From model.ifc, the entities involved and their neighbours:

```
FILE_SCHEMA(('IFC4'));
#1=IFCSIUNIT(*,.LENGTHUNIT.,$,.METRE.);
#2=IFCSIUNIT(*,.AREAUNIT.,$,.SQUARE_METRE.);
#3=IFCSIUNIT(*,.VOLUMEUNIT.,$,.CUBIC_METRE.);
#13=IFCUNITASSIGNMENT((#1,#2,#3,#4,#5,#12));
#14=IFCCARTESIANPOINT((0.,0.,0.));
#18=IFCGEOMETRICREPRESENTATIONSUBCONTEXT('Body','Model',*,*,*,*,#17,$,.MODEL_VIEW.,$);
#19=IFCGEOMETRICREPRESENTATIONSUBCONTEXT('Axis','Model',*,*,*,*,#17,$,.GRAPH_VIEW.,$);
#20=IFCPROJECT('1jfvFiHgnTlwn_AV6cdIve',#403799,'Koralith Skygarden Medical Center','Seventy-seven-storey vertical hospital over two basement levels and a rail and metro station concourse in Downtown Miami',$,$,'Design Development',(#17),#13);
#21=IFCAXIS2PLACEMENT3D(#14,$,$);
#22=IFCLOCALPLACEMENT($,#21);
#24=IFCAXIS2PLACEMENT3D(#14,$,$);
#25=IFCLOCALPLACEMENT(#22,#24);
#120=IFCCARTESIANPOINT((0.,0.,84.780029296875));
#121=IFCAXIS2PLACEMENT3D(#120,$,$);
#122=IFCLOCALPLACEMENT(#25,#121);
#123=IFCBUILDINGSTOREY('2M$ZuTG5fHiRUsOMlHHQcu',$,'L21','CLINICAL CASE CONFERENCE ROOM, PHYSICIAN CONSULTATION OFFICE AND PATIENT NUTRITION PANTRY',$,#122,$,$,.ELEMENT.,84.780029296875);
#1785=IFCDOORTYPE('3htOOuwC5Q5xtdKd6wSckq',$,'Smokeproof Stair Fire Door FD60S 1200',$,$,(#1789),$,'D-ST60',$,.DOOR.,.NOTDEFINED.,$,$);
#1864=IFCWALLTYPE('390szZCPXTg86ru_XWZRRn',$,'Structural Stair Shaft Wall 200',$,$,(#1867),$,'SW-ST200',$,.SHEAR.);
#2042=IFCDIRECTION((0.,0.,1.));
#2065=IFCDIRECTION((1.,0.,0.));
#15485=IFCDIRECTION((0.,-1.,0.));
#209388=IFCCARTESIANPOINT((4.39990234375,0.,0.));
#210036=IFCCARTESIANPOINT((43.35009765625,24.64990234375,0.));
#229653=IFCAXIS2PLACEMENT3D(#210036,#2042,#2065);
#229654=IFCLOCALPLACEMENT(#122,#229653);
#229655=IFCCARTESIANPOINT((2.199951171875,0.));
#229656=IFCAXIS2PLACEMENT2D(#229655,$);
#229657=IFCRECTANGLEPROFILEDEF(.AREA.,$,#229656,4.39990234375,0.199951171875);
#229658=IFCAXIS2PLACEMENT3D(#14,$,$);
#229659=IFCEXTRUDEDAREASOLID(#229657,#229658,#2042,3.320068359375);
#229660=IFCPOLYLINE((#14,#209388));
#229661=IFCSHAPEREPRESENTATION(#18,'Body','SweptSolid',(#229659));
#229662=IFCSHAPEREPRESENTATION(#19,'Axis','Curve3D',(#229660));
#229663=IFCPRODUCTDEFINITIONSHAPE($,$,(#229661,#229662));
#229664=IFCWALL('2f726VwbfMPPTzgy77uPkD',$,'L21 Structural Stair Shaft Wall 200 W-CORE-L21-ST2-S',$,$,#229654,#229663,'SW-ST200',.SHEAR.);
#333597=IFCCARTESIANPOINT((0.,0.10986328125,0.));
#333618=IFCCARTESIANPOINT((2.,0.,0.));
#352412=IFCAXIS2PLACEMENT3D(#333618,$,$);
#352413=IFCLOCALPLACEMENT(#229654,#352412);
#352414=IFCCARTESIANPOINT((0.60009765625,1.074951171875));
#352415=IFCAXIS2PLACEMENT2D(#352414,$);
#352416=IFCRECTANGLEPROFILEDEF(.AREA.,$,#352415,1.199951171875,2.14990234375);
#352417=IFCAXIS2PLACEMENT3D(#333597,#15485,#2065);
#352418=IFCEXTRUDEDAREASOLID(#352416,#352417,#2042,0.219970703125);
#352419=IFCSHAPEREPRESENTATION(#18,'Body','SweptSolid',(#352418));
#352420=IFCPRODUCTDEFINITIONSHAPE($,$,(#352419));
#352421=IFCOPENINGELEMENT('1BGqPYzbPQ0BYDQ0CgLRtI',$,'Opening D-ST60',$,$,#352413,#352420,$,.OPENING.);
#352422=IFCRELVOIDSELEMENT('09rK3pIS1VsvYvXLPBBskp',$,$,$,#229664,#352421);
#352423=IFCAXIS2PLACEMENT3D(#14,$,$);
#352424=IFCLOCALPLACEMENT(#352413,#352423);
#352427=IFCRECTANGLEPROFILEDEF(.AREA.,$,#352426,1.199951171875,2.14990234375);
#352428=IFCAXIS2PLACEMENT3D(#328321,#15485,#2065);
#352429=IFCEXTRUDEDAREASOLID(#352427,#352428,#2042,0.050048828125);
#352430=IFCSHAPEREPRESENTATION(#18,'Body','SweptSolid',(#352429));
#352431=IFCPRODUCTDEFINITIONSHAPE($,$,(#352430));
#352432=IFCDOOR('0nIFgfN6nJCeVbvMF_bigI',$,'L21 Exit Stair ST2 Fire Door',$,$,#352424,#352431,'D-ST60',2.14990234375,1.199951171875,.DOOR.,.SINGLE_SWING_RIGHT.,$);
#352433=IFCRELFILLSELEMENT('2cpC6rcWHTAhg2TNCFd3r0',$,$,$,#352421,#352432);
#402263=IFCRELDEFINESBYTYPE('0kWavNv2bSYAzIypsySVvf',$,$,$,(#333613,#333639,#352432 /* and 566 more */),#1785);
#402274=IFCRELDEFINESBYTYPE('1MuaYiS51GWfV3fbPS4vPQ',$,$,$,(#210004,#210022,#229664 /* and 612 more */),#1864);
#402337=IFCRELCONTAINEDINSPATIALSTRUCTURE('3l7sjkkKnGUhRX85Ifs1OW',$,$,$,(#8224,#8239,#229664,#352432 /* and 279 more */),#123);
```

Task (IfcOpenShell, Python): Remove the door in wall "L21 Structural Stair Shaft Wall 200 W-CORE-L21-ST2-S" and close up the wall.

```python
import ifcopenshell
import ifcopenshell.api.feature
import ifcopenshell.api.root
import ifcopenshell.geom
import ifcopenshell.util.shape

model = ifcopenshell.open("model.ifc")
settings = ifcopenshell.geom.settings()


def volume(element):
    """Net volume in cubic metres, openings subtracted."""
    shape = ifcopenshell.geom.create_shape(settings, element)
    return ifcopenshell.util.shape.get_volume(shape.geometry)


door = model.by_id(352432)
opening = door.FillsVoids[0].RelatingOpeningElement
wall = opening.VoidsElements[0].RelatingBuildingElement
before = volume(wall)

ifcopenshell.api.root.remove_product(model, product=door)
ifcopenshell.api.feature.remove_feature(model, feature=opening)

after = volume(wall)

print(f"wall volume {before:.3f} -> {after:.3f} m3")

model.write("model_edited.ifc")
```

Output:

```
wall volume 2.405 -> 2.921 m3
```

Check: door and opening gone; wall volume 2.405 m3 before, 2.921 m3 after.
